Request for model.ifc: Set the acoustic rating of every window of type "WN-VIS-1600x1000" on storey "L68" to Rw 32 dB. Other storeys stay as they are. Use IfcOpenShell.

First a look at what the model holds.

```python
import ifcopenshell
import ifcopenshell.util.element

model = ifcopenshell.open("model.ifc")
print(model.schema)
storey = next(s for s in model.by_type("IfcBuildingStorey") if s.Name == "L68")
windows = [e for e in ifcopenshell.util.element.get_decomposition(storey) if e.is_a("IfcWindow")]
seen = {}
for e in windows:
    element_type = ifcopenshell.util.element.get_type(e)
    key = (element_type.Name if element_type != e and element_type else None, ifcopenshell.util.element.get_pset(e, "Pset_WindowCommon", "AcousticRating"))
    seen[key] = seen.get(key, 0) + 1
for (name, value), count in sorted(seen.items(), key=str):
    print(count, "x", name, "|", value)
```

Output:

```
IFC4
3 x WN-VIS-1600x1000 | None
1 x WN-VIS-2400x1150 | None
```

```python
import ifcopenshell
import ifcopenshell.api.pset
import ifcopenshell.util.element

model = ifcopenshell.open("model.ifc")

storey = next(s for s in model.by_type("IfcBuildingStorey") if s.Name == "L68")
windows = [e for e in ifcopenshell.util.element.get_decomposition(storey) if e.is_a("IfcWindow")]

count = 0
for e in windows:
    element_type = ifcopenshell.util.element.get_type(e)
    if element_type in (None, e) or element_type.Name != "WN-VIS-1600x1000":
        continue
    found = ifcopenshell.util.element.get_pset(e, "Pset_WindowCommon", should_inherit=False)
    if found:
        pset = model.by_id(found["id"])
        if len(ifcopenshell.util.element.get_elements_by_pset(pset)) > 1:
            pset = ifcopenshell.api.pset.unshare_pset(model, products=[e], pset=pset)[0]
    else:
        pset = ifcopenshell.api.pset.add_pset(model, product=e, name="Pset_WindowCommon")
    ifcopenshell.api.pset.edit_pset(model, pset=pset, properties={"AcousticRating": "Rw 32 dB"})
    count += 1

print(count, "windows updated")

model.write("model_v2.ifc")
```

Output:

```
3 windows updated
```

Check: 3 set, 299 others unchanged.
